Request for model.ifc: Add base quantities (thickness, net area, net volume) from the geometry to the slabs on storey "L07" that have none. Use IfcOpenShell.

First a look at what the model holds.

```python
import ifcopenshell
import ifcopenshell.util.element
import ifcopenshell.util.unit

model = ifcopenshell.open("model.ifc")
print(model.schema)
for unit_type in ("LENGTHUNIT", "AREAUNIT", "VOLUMEUNIT"):
    print(unit_type, ifcopenshell.util.unit.calculate_unit_scale(model, unit_type))
storey = next(s for s in model.by_type("IfcBuildingStorey") if s.Name == "L07")
slabs = [e for e in ifcopenshell.util.element.get_decomposition(storey) if e.is_a("IfcSlab")]
for e in sorted(slabs, key=lambda e: e.id()):
    print(e.id(), e.is_a(), e.Name, list(ifcopenshell.util.element.get_psets(e, qtos_only=True)), sep=" | ")
```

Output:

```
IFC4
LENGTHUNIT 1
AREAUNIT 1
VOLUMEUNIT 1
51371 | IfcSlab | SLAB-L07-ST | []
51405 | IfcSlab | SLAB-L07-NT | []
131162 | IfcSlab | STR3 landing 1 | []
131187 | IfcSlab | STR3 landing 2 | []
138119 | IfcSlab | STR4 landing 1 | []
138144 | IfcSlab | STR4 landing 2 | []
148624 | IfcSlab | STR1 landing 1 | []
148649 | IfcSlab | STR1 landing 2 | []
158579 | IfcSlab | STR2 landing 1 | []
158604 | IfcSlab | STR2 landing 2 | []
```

```python
import ifcopenshell
import ifcopenshell.api.pset
import ifcopenshell.geom
import ifcopenshell.util.element
import ifcopenshell.util.shape
import ifcopenshell.util.unit

model = ifcopenshell.open("model.ifc")
unit_scale = ifcopenshell.util.unit.calculate_unit_scale(model)
area_scale = ifcopenshell.util.unit.calculate_unit_scale(model, "AREAUNIT")
volume_scale = ifcopenshell.util.unit.calculate_unit_scale(model, "VOLUMEUNIT")
settings = ifcopenshell.geom.settings()

storey = next(s for s in model.by_type("IfcBuildingStorey") if s.Name == "L07")
slabs = [e for e in ifcopenshell.util.element.get_decomposition(storey) if e.is_a("IfcSlab")]

for e in sorted(slabs, key=lambda e: e.id()):
    if ifcopenshell.util.element.get_psets(e, qtos_only=True, should_inherit=False):
        continue
    # Geometry comes back in metres, in the element's own axes.
    shape = ifcopenshell.geom.create_shape(settings, e)
    values = {
        "Width": ifcopenshell.util.shape.get_z(shape.geometry) / unit_scale,
        "NetArea": ifcopenshell.util.shape.get_footprint_area(shape.geometry) / area_scale,
        "NetVolume": ifcopenshell.util.shape.get_volume(shape.geometry) / volume_scale,
    }
    qto = ifcopenshell.api.pset.add_qto(model, product=e, name="Qto_SlabBaseQuantities")
    ifcopenshell.api.pset.edit_qto(model, qto=qto, properties=values)
    print(e.id(), {k: round(v, 3) for k, v in values.items()})

model.write("model-out.ifc")
```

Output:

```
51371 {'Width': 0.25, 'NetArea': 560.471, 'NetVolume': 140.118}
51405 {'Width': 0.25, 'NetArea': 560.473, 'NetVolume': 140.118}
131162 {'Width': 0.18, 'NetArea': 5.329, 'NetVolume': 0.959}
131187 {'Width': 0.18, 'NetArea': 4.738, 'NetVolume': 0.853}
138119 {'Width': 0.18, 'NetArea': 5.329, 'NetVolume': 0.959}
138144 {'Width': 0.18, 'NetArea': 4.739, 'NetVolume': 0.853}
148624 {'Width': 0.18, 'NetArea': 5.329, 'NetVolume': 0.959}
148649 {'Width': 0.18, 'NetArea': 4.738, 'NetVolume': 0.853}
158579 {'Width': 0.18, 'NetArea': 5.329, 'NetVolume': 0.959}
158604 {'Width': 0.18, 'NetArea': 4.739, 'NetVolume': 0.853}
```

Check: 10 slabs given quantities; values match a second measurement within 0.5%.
